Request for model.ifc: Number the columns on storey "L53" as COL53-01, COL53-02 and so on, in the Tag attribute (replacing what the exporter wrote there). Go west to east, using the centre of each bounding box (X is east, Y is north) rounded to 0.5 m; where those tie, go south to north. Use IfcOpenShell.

First a look at what the model holds.

```python
import ifcopenshell
import ifcopenshell.util.element
import ifcopenshell.util.placement

model = ifcopenshell.open("model.ifc")
print(model.schema)
storey = next(s for s in model.by_type("IfcBuildingStorey") if s.Name == "L53")
columns = [e for e in ifcopenshell.util.element.get_decomposition(storey) if e.is_a("IfcColumn")]
for e in sorted(columns, key=lambda e: e.id()):
    origin = ifcopenshell.util.placement.get_local_placement(e.ObjectPlacement)[:3, 3]
    print(e.id(), e.Tag, e.Name, origin.round(2) + 0.0, sep=" | ")
```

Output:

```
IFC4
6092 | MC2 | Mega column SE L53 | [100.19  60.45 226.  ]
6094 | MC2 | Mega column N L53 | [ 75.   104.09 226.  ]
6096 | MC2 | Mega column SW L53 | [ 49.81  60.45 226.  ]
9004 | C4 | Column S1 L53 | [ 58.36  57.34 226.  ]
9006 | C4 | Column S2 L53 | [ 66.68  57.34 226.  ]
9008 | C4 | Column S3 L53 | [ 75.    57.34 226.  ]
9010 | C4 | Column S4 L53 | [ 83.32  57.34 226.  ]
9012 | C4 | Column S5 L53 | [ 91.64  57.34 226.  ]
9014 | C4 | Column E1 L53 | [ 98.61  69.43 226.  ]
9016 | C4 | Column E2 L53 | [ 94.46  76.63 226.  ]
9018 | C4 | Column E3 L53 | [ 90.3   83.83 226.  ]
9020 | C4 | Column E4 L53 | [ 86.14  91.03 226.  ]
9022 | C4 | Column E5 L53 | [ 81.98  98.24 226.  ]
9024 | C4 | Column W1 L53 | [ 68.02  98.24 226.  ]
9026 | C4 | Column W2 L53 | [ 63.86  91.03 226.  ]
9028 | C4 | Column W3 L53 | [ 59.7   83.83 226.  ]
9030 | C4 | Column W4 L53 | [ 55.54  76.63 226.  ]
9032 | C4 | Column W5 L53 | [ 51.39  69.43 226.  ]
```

```python
import ifcopenshell
import ifcopenshell.geom
import ifcopenshell.util.element
import ifcopenshell.util.shape

model = ifcopenshell.open("model.ifc")
settings = ifcopenshell.geom.settings()
settings.set("use-world-coords", True)


def centre(element):
    shape = ifcopenshell.geom.create_shape(settings, element)
    return ifcopenshell.util.shape.get_bbox_centroid(shape.geometry)


storey = next(s for s in model.by_type("IfcBuildingStorey") if s.Name == "L53")
columns = [e for e in ifcopenshell.util.element.get_decomposition(storey) if e.is_a("IfcColumn")]

# Insertion points can sit at a corner or the storey origin, so sort by the geometry (in metres).
centres = {e: centre(e) for e in columns}
columns.sort(key=lambda e: (round(centres[e][0] / 0.5), centres[e][1]))

for i, e in enumerate(columns, start=1):
    number = f"COL53-{i:02d}"
    e.Tag = number
    print(e.id(), number)

model.write("model_edited.ifc")
```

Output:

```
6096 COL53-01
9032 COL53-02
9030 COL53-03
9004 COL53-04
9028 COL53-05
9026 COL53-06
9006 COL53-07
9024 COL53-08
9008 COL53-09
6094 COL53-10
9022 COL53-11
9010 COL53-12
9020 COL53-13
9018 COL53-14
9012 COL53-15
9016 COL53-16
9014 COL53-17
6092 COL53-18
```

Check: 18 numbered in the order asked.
